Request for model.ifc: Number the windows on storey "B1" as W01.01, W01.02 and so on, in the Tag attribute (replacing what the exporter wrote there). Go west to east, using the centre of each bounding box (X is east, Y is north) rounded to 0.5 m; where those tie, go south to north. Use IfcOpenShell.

First a look at what the model holds.

```python
import ifcopenshell
import ifcopenshell.util.element
import ifcopenshell.util.placement

model = ifcopenshell.open("model.ifc")
print(model.schema)
storey = next(s for s in model.by_type("IfcBuildingStorey") if s.Name == "B1")
windows = [e for e in ifcopenshell.util.element.get_decomposition(storey) if e.is_a("IfcWindow")]
for e in sorted(windows, key=lambda e: e.id()):
    origin = ifcopenshell.util.placement.get_local_placement(e.ObjectPlacement)[:3, 3]
    print(e.id(), e.Tag, e.Name, origin.round(2) + 0.0, sep=" | ")
```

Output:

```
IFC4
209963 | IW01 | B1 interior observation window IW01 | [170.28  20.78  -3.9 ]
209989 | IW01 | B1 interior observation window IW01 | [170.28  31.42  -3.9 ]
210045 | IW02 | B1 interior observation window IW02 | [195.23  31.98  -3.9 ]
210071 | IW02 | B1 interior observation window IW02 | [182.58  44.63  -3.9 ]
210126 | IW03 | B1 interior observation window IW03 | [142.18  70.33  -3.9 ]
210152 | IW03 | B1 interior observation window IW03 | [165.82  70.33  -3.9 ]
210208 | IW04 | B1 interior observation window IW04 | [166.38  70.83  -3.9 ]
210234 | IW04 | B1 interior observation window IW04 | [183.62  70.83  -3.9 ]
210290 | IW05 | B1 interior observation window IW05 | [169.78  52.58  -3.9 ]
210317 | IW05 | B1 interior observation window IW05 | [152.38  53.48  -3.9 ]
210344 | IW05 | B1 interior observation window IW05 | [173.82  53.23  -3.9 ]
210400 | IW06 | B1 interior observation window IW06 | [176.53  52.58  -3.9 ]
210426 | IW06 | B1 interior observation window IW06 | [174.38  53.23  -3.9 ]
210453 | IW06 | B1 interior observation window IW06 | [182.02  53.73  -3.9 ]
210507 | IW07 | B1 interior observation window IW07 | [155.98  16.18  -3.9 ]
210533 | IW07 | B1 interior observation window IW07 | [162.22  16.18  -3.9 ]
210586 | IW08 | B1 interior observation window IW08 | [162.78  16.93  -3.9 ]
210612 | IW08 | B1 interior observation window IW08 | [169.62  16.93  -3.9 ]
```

```python
import ifcopenshell
import ifcopenshell.geom
import ifcopenshell.util.element
import ifcopenshell.util.shape

model = ifcopenshell.open("model.ifc")
settings = ifcopenshell.geom.settings()
settings.set("use-world-coords", True)


def centre(element):
    shape = ifcopenshell.geom.create_shape(settings, element)
    return ifcopenshell.util.shape.get_bbox_centroid(shape.geometry)


storey = next(s for s in model.by_type("IfcBuildingStorey") if s.Name == "B1")
windows = [e for e in ifcopenshell.util.element.get_decomposition(storey) if e.is_a("IfcWindow")]

# Insertion points can sit at a corner or the storey origin, so sort by the geometry (in metres).
centres = {e: centre(e) for e in windows}
windows.sort(key=lambda e: (round(centres[e][0] / 0.5), centres[e][1]))

for i, e in enumerate(windows, start=1):
    number = f"W01.{i:02d}"
    e.Tag = number
    print(e.id(), number)

model.write("model_updated.ifc")
```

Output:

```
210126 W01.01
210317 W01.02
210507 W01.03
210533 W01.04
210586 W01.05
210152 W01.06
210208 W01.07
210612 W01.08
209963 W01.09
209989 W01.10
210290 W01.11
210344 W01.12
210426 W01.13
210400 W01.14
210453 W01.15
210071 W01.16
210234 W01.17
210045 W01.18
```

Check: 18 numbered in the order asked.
